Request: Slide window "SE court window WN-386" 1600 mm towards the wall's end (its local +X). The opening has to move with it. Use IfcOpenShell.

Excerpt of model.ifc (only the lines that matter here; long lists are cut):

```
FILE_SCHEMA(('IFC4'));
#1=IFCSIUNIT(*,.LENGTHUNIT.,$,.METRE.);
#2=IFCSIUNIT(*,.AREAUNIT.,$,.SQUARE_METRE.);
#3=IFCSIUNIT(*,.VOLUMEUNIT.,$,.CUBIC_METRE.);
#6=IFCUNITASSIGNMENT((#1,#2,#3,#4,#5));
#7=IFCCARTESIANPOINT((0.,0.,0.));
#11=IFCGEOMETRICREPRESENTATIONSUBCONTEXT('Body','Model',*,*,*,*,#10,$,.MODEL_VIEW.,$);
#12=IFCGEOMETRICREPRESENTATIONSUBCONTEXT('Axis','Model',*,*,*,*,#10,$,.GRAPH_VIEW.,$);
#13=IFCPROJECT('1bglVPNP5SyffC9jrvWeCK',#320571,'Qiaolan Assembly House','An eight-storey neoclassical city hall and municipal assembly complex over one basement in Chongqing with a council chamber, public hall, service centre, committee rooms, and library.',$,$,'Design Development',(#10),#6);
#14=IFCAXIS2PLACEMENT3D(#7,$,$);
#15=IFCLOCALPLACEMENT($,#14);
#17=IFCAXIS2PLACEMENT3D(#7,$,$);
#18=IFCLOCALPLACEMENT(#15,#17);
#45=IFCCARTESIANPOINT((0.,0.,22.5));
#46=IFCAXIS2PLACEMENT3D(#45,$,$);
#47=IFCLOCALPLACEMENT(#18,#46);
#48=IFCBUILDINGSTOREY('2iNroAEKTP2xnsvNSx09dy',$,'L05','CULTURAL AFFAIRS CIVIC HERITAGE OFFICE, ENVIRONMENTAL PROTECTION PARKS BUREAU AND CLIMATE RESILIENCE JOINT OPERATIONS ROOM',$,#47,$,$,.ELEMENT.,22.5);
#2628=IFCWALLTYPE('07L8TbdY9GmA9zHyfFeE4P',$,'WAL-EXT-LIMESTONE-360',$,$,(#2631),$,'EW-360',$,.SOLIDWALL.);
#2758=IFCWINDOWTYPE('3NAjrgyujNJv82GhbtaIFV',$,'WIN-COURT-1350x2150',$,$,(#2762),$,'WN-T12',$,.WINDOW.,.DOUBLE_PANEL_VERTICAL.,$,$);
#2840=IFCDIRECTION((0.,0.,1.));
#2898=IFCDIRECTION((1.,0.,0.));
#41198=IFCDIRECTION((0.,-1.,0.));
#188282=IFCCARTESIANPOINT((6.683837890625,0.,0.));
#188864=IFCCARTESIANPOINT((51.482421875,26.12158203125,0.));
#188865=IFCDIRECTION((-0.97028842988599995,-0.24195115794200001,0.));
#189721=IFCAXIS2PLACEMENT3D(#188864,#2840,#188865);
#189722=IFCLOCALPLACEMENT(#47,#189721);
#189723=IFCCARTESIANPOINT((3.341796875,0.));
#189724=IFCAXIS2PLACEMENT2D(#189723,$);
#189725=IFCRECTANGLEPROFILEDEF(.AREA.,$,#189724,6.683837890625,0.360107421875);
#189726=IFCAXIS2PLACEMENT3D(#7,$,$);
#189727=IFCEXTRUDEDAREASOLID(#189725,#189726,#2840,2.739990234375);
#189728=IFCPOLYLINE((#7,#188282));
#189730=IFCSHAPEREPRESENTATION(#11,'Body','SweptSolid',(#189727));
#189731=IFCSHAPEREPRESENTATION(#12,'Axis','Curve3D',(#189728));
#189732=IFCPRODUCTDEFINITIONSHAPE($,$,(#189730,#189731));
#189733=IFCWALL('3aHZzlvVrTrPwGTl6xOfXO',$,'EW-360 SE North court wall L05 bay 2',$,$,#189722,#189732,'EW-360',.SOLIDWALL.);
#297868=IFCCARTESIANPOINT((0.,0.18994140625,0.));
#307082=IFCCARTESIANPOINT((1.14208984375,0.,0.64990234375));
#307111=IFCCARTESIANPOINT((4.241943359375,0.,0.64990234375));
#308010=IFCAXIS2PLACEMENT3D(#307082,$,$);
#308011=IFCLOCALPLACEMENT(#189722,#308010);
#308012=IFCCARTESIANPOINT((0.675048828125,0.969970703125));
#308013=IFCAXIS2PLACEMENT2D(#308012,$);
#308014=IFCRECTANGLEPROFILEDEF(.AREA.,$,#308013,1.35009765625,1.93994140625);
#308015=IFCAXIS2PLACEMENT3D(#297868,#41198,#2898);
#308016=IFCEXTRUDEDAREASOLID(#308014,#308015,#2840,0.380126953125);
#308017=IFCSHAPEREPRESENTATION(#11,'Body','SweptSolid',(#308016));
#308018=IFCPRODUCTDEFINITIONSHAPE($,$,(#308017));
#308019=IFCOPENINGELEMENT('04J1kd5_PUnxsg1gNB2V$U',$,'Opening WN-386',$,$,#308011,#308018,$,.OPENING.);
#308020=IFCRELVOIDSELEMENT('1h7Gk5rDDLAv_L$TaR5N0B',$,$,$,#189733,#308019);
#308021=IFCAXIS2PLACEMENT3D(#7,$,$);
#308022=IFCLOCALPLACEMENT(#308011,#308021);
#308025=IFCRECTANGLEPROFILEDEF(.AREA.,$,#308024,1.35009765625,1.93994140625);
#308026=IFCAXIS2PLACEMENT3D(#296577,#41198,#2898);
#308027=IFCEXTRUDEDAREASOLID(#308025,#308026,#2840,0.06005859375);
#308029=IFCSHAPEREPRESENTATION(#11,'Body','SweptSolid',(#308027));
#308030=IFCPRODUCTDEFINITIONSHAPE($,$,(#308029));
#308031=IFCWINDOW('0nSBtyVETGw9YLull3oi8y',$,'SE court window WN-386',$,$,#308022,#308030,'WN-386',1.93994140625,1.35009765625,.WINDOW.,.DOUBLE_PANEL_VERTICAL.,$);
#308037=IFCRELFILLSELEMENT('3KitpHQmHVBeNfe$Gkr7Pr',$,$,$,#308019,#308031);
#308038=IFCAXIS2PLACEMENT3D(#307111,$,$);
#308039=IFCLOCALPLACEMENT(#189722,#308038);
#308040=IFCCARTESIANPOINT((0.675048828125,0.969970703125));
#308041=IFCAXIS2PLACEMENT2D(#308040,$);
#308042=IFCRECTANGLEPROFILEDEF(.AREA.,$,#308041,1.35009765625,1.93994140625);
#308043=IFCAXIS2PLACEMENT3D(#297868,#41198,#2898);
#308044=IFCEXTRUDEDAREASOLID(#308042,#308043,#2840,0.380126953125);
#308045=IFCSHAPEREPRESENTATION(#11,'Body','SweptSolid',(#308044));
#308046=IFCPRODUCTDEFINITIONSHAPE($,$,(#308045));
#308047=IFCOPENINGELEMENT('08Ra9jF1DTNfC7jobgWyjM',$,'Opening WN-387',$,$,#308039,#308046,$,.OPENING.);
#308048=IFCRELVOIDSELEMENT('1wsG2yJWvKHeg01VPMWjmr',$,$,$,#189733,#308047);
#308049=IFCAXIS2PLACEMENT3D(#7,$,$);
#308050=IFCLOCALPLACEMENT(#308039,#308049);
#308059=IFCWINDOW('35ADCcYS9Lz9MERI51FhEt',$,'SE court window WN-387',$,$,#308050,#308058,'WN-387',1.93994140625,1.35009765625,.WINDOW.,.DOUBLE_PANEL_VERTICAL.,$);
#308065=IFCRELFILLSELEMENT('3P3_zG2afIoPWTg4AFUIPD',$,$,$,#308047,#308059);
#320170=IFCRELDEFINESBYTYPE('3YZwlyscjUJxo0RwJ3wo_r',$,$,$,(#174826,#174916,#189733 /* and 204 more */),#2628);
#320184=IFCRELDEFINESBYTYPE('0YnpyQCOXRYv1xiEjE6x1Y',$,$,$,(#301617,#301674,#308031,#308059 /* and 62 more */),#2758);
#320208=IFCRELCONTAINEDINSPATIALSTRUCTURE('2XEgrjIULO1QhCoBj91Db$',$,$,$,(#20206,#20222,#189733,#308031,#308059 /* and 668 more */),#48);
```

```python
import ifcopenshell
import ifcopenshell.api.geometry
import ifcopenshell.util.placement

model = ifcopenshell.open("model.ifc")

window = model.by_id(308031)
opening = window.FillsVoids[0].RelatingOpeningElement
wall = opening.VoidsElements[0].RelatingBuildingElement

wall_matrix = ifcopenshell.util.placement.get_local_placement(wall.ObjectPlacement)
shift = wall_matrix[:3, 0] * 1.6
before = ifcopenshell.util.placement.get_local_placement(window.ObjectPlacement)[:3, 3].copy()

# The window is placed relative to its opening, so it follows when the opening moves.
matrix = ifcopenshell.util.placement.get_local_placement(opening.ObjectPlacement)
matrix[:3, 3] += shift
ifcopenshell.api.geometry.edit_object_placement(
    model, product=opening, matrix=matrix, is_si=False, should_transform_children=True
)

after = ifcopenshell.util.placement.get_local_placement(window.ObjectPlacement)[:3, 3]
print("window moved by", (after - before).round(3) + 0.0)

model.write("model-out.ifc")
```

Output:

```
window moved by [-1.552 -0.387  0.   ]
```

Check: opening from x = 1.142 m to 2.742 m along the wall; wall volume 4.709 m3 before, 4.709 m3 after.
